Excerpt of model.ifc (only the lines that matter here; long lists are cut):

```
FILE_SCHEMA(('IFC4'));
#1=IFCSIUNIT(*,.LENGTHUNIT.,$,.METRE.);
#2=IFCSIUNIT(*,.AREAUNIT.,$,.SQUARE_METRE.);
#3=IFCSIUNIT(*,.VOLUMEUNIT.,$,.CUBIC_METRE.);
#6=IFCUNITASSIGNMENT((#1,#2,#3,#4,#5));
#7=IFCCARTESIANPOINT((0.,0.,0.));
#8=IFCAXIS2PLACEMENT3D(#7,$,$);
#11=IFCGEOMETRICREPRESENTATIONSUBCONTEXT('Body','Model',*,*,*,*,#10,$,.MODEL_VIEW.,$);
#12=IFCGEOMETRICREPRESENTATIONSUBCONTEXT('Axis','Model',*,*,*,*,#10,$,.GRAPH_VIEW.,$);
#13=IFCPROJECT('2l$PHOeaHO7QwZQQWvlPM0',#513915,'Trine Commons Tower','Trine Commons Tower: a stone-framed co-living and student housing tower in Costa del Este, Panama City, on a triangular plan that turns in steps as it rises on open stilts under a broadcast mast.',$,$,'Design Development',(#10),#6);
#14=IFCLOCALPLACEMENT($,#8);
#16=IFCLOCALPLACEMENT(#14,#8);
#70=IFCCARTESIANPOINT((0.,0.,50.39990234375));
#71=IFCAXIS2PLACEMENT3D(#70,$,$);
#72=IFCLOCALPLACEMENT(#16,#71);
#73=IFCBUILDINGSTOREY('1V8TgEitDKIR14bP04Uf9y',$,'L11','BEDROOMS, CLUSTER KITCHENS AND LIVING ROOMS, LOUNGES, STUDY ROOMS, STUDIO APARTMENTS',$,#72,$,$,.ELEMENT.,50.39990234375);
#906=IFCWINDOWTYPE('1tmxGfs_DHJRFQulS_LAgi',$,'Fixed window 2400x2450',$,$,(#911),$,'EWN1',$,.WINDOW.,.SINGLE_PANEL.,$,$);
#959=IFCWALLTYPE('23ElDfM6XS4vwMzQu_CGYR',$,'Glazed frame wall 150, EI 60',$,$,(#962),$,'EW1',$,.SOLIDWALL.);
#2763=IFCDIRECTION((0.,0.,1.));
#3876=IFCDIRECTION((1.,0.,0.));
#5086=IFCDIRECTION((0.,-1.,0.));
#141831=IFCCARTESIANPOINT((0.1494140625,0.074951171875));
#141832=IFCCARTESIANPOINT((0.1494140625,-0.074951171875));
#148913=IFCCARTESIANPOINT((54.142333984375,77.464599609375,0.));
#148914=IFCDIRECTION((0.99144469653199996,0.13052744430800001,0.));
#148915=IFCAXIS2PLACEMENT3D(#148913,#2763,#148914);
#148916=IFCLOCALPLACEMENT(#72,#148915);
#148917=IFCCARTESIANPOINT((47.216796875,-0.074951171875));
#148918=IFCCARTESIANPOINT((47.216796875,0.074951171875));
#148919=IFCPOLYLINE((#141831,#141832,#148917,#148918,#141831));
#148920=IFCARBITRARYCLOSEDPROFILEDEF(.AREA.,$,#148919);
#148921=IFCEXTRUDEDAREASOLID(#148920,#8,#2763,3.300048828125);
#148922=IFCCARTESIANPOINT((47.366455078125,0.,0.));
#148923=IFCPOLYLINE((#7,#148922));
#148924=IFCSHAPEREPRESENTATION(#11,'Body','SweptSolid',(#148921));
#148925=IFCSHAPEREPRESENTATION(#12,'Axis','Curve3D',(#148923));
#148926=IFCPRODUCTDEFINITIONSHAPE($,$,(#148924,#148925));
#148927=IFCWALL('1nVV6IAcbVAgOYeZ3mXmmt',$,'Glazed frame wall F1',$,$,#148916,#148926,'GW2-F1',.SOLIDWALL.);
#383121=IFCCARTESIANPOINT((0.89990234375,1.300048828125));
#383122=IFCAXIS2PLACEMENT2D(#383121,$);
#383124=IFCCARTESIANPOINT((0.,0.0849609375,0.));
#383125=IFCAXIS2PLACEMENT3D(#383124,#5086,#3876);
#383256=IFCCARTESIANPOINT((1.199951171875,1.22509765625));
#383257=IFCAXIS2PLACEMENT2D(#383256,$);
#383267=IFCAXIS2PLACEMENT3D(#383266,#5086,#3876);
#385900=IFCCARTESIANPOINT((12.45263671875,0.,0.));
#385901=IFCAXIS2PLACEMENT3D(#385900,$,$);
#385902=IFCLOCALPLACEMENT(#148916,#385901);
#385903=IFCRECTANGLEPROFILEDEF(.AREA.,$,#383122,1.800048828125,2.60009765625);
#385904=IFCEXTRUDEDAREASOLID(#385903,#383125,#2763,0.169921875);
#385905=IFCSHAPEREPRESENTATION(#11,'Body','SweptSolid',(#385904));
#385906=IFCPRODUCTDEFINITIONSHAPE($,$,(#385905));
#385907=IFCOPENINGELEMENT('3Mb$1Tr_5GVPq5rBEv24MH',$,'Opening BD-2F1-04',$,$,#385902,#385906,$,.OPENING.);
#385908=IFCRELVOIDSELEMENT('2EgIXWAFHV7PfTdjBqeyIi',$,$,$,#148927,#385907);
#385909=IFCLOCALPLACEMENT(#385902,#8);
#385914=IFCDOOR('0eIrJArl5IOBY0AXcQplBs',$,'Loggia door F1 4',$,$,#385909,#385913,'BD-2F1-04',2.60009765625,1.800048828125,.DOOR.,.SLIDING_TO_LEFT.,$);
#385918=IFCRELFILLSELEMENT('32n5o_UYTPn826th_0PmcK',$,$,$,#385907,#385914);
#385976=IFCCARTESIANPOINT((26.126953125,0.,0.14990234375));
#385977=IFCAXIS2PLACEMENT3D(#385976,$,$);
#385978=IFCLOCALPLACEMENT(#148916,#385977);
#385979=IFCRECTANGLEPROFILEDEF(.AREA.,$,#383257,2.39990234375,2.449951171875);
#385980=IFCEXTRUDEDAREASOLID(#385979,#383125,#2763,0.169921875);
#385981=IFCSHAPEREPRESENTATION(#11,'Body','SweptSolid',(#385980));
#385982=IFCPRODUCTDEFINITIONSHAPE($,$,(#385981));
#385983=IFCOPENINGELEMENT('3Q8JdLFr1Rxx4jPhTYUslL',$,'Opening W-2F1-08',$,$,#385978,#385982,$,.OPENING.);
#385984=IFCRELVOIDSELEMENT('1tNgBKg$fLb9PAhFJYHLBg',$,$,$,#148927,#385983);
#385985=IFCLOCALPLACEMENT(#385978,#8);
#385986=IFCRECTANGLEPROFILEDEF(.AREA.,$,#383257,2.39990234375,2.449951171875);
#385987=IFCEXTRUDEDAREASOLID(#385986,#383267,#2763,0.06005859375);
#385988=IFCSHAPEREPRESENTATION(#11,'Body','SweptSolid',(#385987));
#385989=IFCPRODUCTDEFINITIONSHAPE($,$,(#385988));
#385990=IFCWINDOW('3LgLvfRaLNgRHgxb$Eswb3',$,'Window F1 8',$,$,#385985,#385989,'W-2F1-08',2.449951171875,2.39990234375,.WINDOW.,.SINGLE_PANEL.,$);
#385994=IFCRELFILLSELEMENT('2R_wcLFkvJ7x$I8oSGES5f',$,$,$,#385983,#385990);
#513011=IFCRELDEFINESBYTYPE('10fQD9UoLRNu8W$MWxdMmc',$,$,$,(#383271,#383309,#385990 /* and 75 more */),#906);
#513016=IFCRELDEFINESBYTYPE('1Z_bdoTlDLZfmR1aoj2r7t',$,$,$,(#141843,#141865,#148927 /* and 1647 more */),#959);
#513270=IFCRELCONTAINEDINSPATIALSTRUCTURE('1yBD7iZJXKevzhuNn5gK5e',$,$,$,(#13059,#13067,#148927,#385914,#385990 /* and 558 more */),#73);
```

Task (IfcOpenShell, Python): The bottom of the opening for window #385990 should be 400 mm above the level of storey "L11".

```python
import numpy as np
import ifcopenshell
import ifcopenshell.api.geometry
import ifcopenshell.geom
import ifcopenshell.util.element
import ifcopenshell.util.placement
import ifcopenshell.util.shape
import ifcopenshell.util.unit

model = ifcopenshell.open("model.ifc")
unit_scale = ifcopenshell.util.unit.calculate_unit_scale(model)

window = model.by_guid("3LgLvfRaLNgRHgxb$Eswb3")
opening = window.FillsVoids[0].RelatingOpeningElement
storey = ifcopenshell.util.element.get_container(window, ifc_class="IfcBuildingStorey")
level = ifcopenshell.util.placement.get_local_placement(storey.ObjectPlacement)[2, 3]

# The opening's origin need not be at the sill, so measure its lowest point.
shape = ifcopenshell.geom.create_shape(ifcopenshell.geom.settings(), opening)
bottom = ifcopenshell.util.shape.get_shape_bottom_elevation(shape, shape.geometry) / unit_scale
dz = level + 0.4 / unit_scale - bottom

shift = np.array([0.0, 0.0, dz])
# The window is placed relative to its opening, so it follows when the opening moves.
matrix = ifcopenshell.util.placement.get_local_placement(opening.ObjectPlacement)
matrix[:3, 3] += shift
ifcopenshell.api.geometry.edit_object_placement(
    model, product=opening, matrix=matrix, is_si=False, should_transform_children=True
)

print(f"moved by {dz * unit_scale:+.3f} m")

model.write("model_updated.ifc")
```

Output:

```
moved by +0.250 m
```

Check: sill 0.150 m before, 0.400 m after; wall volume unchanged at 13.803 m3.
